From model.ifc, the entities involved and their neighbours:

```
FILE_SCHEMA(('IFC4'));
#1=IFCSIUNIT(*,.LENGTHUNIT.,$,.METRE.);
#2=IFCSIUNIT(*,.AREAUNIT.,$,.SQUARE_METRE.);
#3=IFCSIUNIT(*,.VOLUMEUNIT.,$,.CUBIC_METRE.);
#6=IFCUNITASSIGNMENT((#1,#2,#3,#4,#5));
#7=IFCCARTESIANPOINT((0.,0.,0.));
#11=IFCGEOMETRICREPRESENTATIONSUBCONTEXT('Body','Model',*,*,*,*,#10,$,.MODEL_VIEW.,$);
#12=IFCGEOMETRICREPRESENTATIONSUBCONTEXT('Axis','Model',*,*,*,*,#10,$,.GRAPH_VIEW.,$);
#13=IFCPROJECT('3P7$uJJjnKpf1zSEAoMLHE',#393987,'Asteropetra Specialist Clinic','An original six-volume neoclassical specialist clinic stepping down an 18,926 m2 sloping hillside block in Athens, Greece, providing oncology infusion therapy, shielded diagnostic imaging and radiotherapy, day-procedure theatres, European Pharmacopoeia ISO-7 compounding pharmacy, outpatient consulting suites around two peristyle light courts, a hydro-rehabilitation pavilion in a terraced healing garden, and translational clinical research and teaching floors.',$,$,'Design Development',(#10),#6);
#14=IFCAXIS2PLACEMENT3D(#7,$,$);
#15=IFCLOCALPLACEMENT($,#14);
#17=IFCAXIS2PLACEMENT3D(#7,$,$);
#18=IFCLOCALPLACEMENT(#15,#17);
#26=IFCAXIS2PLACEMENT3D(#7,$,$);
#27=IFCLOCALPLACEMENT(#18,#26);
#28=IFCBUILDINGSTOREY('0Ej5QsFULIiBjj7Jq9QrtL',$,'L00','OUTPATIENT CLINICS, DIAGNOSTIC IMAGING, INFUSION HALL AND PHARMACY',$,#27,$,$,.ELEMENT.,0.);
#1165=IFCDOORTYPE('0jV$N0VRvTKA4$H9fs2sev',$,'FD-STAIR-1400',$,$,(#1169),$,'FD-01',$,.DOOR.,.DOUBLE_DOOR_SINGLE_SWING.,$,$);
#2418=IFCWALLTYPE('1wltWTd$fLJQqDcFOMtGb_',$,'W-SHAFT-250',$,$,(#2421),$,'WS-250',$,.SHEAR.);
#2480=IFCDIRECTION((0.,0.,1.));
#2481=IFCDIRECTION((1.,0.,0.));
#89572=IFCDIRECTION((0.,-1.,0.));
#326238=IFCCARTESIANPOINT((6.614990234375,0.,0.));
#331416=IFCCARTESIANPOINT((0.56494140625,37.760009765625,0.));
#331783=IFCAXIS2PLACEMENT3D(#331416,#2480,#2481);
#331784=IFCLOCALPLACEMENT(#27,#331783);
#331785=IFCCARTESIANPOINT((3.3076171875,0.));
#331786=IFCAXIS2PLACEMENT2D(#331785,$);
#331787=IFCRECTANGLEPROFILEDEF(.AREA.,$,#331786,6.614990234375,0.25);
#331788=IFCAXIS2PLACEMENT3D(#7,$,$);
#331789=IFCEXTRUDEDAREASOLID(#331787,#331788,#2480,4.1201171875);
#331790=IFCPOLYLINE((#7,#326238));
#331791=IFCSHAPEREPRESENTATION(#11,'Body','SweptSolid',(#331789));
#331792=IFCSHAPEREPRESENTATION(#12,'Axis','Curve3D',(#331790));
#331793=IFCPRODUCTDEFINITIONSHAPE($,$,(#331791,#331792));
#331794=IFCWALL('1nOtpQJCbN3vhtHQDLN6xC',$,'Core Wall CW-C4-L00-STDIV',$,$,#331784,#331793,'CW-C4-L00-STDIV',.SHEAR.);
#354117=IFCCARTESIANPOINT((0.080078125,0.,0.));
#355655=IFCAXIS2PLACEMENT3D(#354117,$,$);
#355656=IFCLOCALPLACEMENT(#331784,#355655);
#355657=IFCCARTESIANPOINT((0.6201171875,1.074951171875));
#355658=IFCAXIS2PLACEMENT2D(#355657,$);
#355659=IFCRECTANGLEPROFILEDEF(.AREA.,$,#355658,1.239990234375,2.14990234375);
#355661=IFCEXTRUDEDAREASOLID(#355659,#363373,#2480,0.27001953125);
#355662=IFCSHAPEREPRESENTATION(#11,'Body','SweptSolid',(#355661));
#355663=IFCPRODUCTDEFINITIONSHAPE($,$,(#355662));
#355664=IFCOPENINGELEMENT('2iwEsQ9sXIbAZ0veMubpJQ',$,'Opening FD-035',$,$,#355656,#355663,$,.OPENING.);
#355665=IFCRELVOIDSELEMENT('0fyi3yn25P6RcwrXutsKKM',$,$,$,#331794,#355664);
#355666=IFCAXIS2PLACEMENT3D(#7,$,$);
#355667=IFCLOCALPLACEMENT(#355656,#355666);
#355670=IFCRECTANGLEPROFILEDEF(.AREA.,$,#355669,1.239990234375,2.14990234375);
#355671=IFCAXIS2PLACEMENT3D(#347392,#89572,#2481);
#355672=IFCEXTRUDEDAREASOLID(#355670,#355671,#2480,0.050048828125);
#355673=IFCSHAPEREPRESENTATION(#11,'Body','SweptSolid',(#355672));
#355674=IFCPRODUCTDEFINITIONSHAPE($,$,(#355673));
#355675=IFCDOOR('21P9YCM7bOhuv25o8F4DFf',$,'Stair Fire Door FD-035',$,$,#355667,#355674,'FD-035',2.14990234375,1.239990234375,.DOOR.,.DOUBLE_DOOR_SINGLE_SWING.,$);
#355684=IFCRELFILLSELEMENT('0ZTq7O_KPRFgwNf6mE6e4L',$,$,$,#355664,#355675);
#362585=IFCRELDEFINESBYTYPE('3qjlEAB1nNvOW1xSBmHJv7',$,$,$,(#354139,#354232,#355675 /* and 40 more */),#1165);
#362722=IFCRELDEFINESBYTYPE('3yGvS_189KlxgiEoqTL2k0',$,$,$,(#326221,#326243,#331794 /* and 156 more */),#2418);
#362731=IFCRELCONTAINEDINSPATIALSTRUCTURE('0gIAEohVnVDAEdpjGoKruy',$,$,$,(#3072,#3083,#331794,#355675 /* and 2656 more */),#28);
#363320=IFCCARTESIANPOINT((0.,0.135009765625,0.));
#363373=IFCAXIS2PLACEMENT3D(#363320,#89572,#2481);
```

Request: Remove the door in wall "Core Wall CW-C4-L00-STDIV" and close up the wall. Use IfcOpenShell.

```python
import ifcopenshell
import ifcopenshell.api.feature
import ifcopenshell.api.root
import ifcopenshell.geom
import ifcopenshell.util.shape

model = ifcopenshell.open("model.ifc")
settings = ifcopenshell.geom.settings()


def volume(element):
    """Net volume in cubic metres, openings subtracted."""
    shape = ifcopenshell.geom.create_shape(settings, element)
    return ifcopenshell.util.shape.get_volume(shape.geometry)


door = model.by_id(355675)
opening = door.FillsVoids[0].RelatingOpeningElement
wall = opening.VoidsElements[0].RelatingBuildingElement
before = volume(wall)

ifcopenshell.api.root.remove_product(model, product=door)
ifcopenshell.api.feature.remove_feature(model, feature=opening)

after = volume(wall)

print(f"wall volume {before:.3f} -> {after:.3f} m3")

model.write("model_rev.ifc")
```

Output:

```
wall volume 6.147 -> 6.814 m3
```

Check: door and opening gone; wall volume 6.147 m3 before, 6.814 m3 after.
